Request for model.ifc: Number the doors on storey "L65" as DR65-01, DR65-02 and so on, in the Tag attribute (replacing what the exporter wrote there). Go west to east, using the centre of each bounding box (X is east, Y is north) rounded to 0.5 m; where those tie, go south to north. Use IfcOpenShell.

First a look at what the model holds.

```python
import ifcopenshell
import ifcopenshell.util.element
import ifcopenshell.util.placement

model = ifcopenshell.open("model.ifc")
print(model.schema)
storey = next(s for s in model.by_type("IfcBuildingStorey") if s.Name == "L65")
doors = [e for e in ifcopenshell.util.element.get_decomposition(storey) if e.is_a("IfcDoor")]
for e in sorted(doors, key=lambda e: e.id()):
    origin = ifcopenshell.util.placement.get_local_placement(e.ObjectPlacement)[:3, 3]
    print(e.id(), e.Tag, e.Name, origin.round(2) + 0.0, sep=" | ")
```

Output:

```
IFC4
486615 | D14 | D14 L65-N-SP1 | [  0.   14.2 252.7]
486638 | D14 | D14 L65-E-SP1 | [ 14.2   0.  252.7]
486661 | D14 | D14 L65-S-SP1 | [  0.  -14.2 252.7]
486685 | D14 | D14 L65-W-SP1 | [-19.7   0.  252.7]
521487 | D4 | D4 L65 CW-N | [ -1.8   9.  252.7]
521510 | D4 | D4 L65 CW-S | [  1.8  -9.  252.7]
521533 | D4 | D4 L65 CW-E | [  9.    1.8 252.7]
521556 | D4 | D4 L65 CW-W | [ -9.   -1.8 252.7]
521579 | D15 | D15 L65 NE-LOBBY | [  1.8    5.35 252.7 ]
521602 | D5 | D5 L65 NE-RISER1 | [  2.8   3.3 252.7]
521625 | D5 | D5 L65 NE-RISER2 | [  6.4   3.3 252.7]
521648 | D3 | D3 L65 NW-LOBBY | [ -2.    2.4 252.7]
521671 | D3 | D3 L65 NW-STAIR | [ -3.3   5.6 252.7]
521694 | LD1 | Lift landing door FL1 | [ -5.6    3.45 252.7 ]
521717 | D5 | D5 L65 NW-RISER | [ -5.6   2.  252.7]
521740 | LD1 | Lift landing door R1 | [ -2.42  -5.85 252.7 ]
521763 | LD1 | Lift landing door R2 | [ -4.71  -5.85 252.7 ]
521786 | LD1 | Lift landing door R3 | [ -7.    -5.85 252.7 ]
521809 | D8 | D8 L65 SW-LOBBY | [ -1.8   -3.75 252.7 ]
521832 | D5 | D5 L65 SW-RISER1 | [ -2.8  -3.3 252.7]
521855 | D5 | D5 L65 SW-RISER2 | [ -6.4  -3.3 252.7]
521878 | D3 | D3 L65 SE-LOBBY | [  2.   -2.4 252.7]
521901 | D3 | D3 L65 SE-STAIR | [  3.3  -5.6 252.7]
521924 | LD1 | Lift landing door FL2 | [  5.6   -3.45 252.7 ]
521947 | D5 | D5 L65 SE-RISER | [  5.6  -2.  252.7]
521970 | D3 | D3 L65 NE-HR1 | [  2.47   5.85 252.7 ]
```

```python
import ifcopenshell
import ifcopenshell.geom
import ifcopenshell.util.element
import ifcopenshell.util.shape

model = ifcopenshell.open("model.ifc")
settings = ifcopenshell.geom.settings()
settings.set("use-world-coords", True)


def centre(element):
    shape = ifcopenshell.geom.create_shape(settings, element)
    return ifcopenshell.util.shape.get_bbox_centroid(shape.geometry)


storey = next(s for s in model.by_type("IfcBuildingStorey") if s.Name == "L65")
doors = [e for e in ifcopenshell.util.element.get_decomposition(storey) if e.is_a("IfcDoor")]

# Insertion points can sit at a corner or the storey origin, so sort by the geometry (in metres).
centres = {e: centre(e) for e in doors}
doors.sort(key=lambda e: (round(centres[e][0] / 0.5), centres[e][1]))

for i, e in enumerate(doors, start=1):
    number = f"DR65-{i:02d}"
    e.Tag = number
    print(e.id(), number)

model.write("model-out.ifc")
```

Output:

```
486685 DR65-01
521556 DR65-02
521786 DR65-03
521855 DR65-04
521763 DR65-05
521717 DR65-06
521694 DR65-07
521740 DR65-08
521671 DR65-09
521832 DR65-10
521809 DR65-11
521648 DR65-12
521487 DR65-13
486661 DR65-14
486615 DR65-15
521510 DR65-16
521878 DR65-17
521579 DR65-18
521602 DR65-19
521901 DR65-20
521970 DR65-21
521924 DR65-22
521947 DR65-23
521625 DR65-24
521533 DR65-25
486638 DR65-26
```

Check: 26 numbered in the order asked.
